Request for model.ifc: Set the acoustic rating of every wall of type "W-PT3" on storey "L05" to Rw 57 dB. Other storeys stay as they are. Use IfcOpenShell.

First a look at what the model holds.

```python
import ifcopenshell
import ifcopenshell.util.element

model = ifcopenshell.open("model.ifc")
print(model.schema)
storey = next(s for s in model.by_type("IfcBuildingStorey") if s.Name == "L05")
walls = [e for e in ifcopenshell.util.element.get_decomposition(storey) if e.is_a("IfcWall")]
seen = {}
for e in walls:
    element_type = ifcopenshell.util.element.get_type(e)
    key = (element_type.Name if element_type != e and element_type else None, ifcopenshell.util.element.get_pset(e, "Pset_WallCommon", "AcousticRating"))
    seen[key] = seen.get(key, 0) + 1
for (name, value), count in sorted(seen.items(), key=str):
    print(count, "x", name, "|", value)
```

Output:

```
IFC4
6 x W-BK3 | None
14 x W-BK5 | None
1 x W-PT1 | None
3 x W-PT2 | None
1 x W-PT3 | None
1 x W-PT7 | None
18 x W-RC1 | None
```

```python
import ifcopenshell
import ifcopenshell.api.pset
import ifcopenshell.util.element

model = ifcopenshell.open("model.ifc")

storey = next(s for s in model.by_type("IfcBuildingStorey") if s.Name == "L05")
walls = [e for e in ifcopenshell.util.element.get_decomposition(storey) if e.is_a("IfcWall")]

count = 0
for e in walls:
    element_type = ifcopenshell.util.element.get_type(e)
    if element_type in (None, e) or element_type.Name != "W-PT3":
        continue
    # add_pset returns the element's existing set when there is one.
    pset = ifcopenshell.api.pset.add_pset(model, product=e, name="Pset_WallCommon")
    ifcopenshell.api.pset.edit_pset(model, pset=pset, properties={"AcousticRating": "Rw 57 dB"})
    count += 1

print(count, "walls updated")

model.write("model_v2.ifc")
```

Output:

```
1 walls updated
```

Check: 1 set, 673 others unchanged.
